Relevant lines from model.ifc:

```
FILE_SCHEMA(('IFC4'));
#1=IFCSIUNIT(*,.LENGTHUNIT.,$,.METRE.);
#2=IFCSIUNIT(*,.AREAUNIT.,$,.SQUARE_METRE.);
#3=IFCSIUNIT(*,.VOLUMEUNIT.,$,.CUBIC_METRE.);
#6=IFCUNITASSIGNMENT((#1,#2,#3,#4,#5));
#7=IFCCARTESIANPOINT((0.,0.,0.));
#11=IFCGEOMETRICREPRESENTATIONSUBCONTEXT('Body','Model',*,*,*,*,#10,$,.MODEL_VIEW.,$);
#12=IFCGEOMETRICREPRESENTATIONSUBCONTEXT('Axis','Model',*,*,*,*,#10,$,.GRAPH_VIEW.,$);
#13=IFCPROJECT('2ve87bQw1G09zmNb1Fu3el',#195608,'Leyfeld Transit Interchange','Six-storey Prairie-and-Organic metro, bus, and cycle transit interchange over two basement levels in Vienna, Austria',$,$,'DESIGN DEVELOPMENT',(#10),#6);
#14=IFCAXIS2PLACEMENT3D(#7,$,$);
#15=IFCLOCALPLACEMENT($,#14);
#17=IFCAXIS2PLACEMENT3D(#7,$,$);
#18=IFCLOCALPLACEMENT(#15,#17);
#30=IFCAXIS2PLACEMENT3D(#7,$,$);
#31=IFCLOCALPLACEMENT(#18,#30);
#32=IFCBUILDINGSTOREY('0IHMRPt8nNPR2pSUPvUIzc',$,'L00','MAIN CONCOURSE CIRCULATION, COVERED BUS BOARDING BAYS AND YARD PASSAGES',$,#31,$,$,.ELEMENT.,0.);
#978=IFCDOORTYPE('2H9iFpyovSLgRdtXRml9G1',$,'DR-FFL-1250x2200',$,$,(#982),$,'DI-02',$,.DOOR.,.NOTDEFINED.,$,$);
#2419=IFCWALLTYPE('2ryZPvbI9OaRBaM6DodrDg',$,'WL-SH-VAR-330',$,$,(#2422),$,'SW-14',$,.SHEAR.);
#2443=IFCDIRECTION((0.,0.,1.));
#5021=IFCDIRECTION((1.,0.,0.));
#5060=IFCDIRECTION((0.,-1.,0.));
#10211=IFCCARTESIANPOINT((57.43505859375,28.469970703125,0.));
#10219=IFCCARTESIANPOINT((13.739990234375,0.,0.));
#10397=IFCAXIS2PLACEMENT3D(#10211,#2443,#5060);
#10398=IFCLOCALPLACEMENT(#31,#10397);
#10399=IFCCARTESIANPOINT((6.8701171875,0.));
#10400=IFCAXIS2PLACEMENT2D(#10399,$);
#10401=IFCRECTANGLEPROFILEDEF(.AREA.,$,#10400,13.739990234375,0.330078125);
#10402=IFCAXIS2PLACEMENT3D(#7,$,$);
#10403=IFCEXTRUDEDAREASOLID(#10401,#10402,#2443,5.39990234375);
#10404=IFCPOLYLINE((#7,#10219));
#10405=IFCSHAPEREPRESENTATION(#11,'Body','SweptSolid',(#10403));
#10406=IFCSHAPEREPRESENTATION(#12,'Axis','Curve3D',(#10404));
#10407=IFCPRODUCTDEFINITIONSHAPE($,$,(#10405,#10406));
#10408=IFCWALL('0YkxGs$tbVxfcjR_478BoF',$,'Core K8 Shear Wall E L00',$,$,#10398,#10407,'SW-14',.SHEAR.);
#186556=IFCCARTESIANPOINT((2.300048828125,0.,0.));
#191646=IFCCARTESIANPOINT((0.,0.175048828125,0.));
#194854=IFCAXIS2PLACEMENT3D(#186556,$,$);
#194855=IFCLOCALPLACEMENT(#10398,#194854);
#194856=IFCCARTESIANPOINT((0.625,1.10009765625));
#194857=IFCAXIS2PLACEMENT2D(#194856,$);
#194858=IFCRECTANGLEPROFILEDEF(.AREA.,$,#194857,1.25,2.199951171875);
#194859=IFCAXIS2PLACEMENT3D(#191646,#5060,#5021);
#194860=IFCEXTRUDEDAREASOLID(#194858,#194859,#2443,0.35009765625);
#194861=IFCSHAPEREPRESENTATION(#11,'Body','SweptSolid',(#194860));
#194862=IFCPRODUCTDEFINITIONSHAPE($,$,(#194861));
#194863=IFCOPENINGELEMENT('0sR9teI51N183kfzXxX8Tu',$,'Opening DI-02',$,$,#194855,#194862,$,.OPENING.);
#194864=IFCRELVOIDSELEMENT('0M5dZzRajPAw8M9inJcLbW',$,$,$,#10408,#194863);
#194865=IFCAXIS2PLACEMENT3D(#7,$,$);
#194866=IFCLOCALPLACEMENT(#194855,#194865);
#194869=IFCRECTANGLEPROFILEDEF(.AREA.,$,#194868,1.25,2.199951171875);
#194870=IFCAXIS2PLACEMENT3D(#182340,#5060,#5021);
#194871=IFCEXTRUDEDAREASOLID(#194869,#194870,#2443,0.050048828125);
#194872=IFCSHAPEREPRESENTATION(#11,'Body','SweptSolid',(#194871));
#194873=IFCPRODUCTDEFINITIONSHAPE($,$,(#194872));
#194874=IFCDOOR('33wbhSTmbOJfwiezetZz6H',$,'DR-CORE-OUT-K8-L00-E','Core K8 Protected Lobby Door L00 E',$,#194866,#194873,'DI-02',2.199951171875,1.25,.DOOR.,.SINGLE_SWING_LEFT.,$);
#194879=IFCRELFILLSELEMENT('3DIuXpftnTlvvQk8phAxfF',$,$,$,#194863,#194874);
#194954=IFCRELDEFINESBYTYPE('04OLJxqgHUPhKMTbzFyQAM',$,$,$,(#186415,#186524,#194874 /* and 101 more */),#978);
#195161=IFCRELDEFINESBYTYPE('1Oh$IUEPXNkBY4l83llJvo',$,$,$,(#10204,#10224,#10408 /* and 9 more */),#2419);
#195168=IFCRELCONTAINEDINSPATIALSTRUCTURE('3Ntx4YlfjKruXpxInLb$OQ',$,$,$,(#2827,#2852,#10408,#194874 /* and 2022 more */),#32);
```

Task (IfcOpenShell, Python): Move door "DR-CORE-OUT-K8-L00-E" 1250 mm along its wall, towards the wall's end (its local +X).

```python
import ifcopenshell
import ifcopenshell.api.geometry
import ifcopenshell.util.placement

model = ifcopenshell.open("model.ifc")

door = model.by_id(194874)
opening = door.FillsVoids[0].RelatingOpeningElement
wall = opening.VoidsElements[0].RelatingBuildingElement

wall_matrix = ifcopenshell.util.placement.get_local_placement(wall.ObjectPlacement)
shift = wall_matrix[:3, 0] * 1.25
before = ifcopenshell.util.placement.get_local_placement(door.ObjectPlacement)[:3, 3].copy()

# The door is placed relative to its opening, so it follows when the opening moves.
matrix = ifcopenshell.util.placement.get_local_placement(opening.ObjectPlacement)
matrix[:3, 3] += shift
ifcopenshell.api.geometry.edit_object_placement(
    model, product=opening, matrix=matrix, is_si=False, should_transform_children=True
)

after = ifcopenshell.util.placement.get_local_placement(door.ObjectPlacement)[:3, 3]
print("door moved by", (after - before).round(3) + 0.0)

model.write("model-out.ifc")
```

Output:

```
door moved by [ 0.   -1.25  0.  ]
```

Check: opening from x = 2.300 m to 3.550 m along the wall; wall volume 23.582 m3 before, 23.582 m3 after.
